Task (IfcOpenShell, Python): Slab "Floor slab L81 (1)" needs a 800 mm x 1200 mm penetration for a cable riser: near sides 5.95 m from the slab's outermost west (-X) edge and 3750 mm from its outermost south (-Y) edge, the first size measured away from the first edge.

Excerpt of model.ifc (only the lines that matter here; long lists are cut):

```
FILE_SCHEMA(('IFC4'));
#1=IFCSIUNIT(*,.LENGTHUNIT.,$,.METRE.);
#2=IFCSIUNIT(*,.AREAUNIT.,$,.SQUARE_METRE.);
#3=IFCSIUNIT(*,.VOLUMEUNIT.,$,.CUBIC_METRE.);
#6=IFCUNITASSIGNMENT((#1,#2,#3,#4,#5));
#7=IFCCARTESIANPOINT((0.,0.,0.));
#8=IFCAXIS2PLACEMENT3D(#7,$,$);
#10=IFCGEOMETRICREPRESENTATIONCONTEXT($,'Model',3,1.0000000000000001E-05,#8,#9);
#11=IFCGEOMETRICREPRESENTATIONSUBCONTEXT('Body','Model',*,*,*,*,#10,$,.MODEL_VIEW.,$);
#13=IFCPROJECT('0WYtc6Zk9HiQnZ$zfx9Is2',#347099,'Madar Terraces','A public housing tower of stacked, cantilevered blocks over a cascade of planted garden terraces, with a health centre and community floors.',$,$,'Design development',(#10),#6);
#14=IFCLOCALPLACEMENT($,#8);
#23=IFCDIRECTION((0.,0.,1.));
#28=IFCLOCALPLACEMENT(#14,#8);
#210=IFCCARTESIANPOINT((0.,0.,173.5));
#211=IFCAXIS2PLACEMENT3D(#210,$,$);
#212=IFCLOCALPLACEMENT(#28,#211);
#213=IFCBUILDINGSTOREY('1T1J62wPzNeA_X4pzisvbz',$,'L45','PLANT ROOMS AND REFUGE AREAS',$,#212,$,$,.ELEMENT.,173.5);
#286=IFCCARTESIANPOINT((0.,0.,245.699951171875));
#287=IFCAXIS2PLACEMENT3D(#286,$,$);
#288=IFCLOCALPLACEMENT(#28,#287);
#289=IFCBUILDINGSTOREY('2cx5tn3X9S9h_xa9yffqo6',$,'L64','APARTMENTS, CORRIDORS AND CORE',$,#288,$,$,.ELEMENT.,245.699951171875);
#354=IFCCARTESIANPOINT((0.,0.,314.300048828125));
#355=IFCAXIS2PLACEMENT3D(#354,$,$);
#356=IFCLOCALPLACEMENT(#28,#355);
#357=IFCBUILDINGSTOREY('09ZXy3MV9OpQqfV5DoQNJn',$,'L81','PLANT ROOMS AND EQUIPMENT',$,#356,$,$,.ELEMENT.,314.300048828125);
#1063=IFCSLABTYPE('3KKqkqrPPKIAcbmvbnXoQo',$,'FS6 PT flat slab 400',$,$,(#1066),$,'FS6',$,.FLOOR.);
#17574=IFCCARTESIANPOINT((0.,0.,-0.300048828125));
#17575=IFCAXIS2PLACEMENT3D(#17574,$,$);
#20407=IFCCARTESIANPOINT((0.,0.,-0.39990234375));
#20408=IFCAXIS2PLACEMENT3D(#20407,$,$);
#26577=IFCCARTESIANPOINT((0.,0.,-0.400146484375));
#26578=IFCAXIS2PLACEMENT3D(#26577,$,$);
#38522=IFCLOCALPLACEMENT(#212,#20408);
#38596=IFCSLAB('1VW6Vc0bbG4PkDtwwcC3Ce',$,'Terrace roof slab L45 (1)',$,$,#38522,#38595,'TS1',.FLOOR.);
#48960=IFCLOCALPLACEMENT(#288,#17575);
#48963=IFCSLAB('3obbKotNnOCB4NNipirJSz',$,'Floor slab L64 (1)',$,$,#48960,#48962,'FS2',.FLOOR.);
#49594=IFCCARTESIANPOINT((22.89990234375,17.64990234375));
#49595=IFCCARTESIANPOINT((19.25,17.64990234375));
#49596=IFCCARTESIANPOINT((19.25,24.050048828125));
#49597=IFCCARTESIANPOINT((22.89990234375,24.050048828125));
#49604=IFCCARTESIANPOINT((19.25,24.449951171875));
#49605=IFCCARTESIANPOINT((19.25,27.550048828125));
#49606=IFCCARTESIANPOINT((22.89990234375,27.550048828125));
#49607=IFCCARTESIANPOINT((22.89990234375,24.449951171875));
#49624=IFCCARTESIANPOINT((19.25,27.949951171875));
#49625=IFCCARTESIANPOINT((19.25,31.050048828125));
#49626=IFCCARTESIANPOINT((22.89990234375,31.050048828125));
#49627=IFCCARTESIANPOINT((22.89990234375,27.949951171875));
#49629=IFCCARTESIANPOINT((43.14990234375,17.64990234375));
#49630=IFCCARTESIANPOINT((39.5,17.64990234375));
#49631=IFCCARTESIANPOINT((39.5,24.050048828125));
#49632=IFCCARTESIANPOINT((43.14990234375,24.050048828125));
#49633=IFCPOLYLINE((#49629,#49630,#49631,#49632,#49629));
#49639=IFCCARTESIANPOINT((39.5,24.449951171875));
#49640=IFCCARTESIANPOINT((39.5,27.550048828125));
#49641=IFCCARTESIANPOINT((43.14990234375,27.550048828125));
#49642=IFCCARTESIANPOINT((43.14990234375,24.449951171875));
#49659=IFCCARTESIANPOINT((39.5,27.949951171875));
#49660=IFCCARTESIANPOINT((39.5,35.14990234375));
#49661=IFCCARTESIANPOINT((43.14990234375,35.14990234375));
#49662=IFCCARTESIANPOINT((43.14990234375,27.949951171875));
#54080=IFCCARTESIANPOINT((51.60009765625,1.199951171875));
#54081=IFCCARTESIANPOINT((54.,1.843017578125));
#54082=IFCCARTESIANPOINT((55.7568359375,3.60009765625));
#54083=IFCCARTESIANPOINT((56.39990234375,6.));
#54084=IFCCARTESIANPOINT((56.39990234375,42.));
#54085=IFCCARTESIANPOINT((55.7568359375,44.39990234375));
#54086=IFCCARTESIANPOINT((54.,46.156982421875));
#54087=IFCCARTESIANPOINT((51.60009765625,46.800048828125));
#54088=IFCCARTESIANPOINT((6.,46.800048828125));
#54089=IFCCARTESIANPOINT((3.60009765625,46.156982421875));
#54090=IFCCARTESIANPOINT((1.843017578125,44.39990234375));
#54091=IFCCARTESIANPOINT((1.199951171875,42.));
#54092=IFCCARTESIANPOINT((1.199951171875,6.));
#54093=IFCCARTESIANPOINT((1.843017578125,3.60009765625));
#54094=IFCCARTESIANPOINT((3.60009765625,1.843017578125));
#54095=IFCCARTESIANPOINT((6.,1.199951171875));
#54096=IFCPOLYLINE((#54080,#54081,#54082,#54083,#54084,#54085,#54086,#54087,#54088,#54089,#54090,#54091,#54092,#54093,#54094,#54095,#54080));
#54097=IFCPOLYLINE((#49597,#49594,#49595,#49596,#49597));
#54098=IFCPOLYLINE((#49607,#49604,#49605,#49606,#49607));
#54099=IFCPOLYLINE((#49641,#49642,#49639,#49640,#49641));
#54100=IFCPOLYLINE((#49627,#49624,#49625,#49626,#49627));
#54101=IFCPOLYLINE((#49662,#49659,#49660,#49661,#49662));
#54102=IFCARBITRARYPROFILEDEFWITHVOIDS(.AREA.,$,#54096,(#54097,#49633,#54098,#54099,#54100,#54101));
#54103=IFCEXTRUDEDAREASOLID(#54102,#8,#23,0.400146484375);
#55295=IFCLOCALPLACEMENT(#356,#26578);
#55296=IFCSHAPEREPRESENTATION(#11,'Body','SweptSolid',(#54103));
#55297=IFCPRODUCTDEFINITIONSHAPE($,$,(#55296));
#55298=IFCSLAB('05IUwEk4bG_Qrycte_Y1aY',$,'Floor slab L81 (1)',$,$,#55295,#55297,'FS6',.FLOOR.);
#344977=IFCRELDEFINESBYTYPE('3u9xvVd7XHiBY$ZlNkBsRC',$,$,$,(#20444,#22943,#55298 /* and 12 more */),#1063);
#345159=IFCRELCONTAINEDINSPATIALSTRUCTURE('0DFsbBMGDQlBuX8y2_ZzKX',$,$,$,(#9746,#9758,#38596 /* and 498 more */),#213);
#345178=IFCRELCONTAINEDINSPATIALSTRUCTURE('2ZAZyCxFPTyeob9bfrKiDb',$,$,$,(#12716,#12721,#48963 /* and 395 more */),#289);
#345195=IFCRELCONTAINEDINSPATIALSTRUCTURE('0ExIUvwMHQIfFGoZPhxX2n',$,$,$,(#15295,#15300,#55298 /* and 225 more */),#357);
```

```python
import numpy as np
import ifcopenshell
import ifcopenshell.api.feature
import ifcopenshell.api.geometry
import ifcopenshell.api.root
import ifcopenshell.geom
import ifcopenshell.util.placement
import ifcopenshell.util.representation
import ifcopenshell.util.shape
import ifcopenshell.util.unit

model = ifcopenshell.open("model.ifc")
unit_scale = ifcopenshell.util.unit.calculate_unit_scale(model)
settings = ifcopenshell.geom.settings()


def volume(element):
    """Net volume in cubic metres, openings subtracted."""
    shape = ifcopenshell.geom.create_shape(settings, element)
    return ifcopenshell.util.shape.get_volume(shape.geometry)


slab = model.by_guid("05IUwEk4bG_Qrycte_Y1aY")
before = volume(slab)

# Extent in the slab's own axes, in metres. The edges named are its -X and -Y sides.
slab_shape = ifcopenshell.geom.create_shape(settings, slab)
vertices = ifcopenshell.util.shape.get_vertices(slab_shape.geometry)
x_min, y_min, bottom = vertices.min(axis=0)
top = vertices[:, 2].max()

opening = ifcopenshell.api.root.create_entity(model, ifc_class="IfcOpeningElement", name="Cable riser opening", predefined_type="OPENING")
context = ifcopenshell.util.representation.get_context(model, "Model", "Body", "MODEL_VIEW")
width, depth = 0.8, 1.2
outline = [(0.0, 0.0), (width, 0.0), (width, depth), (0.0, depth), (0.0, 0.0)]
# Overshoot both faces by 50 mm so the cut is clean.
shape = ifcopenshell.api.geometry.add_slab_representation(
    model, context=context, depth=top - bottom + 0.1, polyline=outline
)
ifcopenshell.api.geometry.assign_representation(model, product=opening, representation=shape)

matrix = ifcopenshell.util.placement.get_local_placement(slab.ObjectPlacement)
matrix[:, 3] = matrix @ np.append(np.array([x_min + 5.95, y_min + 3.75, bottom - 0.05]) / unit_scale, 1.0)
ifcopenshell.api.geometry.edit_object_placement(model, product=opening, matrix=matrix, is_si=False)
ifcopenshell.api.feature.add_feature(model, feature=opening, element=slab)

after = volume(slab)

print(f"slab volume {before:.3f} -> {after:.3f} m3")

model.write("model_edited.ifc")
```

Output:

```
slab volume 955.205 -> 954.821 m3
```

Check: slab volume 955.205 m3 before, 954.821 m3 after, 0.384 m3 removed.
